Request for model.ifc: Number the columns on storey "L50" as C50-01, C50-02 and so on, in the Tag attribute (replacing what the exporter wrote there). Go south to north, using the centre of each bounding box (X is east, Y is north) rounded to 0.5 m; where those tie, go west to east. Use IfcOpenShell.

First a look at what the model holds.

```python
import ifcopenshell
import ifcopenshell.util.element
import ifcopenshell.util.placement

model = ifcopenshell.open("model.ifc")
print(model.schema)
storey = next(s for s in model.by_type("IfcBuildingStorey") if s.Name == "L50")
columns = [e for e in ifcopenshell.util.element.get_decomposition(storey) if e.is_a("IfcColumn")]
for e in sorted(columns, key=lambda e: e.id()):
    origin = ifcopenshell.util.placement.get_local_placement(e.ObjectPlacement)[:3, 3]
    print(e.id(), e.Tag, e.Name, origin.round(2) + 0.0, sep=" | ")
```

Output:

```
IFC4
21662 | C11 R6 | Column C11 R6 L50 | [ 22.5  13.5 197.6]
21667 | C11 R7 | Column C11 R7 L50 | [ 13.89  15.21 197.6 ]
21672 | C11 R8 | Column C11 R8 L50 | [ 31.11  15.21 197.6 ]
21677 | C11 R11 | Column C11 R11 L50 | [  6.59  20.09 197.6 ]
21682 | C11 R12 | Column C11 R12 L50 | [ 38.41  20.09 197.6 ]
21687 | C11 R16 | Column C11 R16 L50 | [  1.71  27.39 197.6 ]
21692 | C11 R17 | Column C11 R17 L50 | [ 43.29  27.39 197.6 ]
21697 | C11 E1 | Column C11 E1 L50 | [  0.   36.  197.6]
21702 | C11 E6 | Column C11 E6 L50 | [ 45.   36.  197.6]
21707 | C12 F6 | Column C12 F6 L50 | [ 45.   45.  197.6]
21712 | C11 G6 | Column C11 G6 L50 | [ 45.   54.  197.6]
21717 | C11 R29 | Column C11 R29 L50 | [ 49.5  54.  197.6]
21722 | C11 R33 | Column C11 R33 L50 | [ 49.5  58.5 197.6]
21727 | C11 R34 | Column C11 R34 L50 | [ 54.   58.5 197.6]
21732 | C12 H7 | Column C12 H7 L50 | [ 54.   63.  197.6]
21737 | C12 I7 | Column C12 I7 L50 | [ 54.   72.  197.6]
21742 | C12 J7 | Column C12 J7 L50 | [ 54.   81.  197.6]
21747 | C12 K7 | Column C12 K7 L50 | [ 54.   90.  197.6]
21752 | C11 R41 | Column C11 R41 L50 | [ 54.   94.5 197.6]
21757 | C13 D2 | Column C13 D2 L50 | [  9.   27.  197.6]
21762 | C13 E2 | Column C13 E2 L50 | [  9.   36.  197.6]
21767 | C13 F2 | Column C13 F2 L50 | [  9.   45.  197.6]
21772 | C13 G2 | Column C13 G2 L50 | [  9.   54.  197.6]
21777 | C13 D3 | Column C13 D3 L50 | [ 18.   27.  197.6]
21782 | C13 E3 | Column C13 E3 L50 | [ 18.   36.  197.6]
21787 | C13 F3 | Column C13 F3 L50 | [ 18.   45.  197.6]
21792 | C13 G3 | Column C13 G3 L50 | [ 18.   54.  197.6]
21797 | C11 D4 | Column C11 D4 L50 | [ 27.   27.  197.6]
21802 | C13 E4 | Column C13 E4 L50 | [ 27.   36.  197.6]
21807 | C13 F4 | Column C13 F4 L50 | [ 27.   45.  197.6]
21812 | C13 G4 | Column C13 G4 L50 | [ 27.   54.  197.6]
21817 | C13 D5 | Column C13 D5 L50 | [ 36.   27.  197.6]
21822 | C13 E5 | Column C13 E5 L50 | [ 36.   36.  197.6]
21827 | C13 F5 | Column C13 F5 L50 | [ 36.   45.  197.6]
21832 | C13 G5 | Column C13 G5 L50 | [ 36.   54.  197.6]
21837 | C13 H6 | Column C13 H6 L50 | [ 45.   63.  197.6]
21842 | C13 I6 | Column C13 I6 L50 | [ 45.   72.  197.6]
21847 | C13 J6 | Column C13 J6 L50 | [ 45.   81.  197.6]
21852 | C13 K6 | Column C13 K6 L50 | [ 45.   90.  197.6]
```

```python
import ifcopenshell
import ifcopenshell.geom
import ifcopenshell.util.element
import ifcopenshell.util.shape

model = ifcopenshell.open("model.ifc")
settings = ifcopenshell.geom.settings()
settings.set("use-world-coords", True)


def centre(element):
    shape = ifcopenshell.geom.create_shape(settings, element)
    return ifcopenshell.util.shape.get_bbox_centroid(shape.geometry)


storey = next(s for s in model.by_type("IfcBuildingStorey") if s.Name == "L50")
columns = [e for e in ifcopenshell.util.element.get_decomposition(storey) if e.is_a("IfcColumn")]

# Insertion points can sit at a corner or the storey origin, so sort by the geometry (in metres).
centres = {e: centre(e) for e in columns}
columns.sort(key=lambda e: (round(centres[e][1] / 0.5), centres[e][0]))

for i, e in enumerate(columns, start=1):
    number = f"C50-{i:02d}"
    e.Tag = number
    print(e.id(), number)

model.write("model_rev.ifc")
```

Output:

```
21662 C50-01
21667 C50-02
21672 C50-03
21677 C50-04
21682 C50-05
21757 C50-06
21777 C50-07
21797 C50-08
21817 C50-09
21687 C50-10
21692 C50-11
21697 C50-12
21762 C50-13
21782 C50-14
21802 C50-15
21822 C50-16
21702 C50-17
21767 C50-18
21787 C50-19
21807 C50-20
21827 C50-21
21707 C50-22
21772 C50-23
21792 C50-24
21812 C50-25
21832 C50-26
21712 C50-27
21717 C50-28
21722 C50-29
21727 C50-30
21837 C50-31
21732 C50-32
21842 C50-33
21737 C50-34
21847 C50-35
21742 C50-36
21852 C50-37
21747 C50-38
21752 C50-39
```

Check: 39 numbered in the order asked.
